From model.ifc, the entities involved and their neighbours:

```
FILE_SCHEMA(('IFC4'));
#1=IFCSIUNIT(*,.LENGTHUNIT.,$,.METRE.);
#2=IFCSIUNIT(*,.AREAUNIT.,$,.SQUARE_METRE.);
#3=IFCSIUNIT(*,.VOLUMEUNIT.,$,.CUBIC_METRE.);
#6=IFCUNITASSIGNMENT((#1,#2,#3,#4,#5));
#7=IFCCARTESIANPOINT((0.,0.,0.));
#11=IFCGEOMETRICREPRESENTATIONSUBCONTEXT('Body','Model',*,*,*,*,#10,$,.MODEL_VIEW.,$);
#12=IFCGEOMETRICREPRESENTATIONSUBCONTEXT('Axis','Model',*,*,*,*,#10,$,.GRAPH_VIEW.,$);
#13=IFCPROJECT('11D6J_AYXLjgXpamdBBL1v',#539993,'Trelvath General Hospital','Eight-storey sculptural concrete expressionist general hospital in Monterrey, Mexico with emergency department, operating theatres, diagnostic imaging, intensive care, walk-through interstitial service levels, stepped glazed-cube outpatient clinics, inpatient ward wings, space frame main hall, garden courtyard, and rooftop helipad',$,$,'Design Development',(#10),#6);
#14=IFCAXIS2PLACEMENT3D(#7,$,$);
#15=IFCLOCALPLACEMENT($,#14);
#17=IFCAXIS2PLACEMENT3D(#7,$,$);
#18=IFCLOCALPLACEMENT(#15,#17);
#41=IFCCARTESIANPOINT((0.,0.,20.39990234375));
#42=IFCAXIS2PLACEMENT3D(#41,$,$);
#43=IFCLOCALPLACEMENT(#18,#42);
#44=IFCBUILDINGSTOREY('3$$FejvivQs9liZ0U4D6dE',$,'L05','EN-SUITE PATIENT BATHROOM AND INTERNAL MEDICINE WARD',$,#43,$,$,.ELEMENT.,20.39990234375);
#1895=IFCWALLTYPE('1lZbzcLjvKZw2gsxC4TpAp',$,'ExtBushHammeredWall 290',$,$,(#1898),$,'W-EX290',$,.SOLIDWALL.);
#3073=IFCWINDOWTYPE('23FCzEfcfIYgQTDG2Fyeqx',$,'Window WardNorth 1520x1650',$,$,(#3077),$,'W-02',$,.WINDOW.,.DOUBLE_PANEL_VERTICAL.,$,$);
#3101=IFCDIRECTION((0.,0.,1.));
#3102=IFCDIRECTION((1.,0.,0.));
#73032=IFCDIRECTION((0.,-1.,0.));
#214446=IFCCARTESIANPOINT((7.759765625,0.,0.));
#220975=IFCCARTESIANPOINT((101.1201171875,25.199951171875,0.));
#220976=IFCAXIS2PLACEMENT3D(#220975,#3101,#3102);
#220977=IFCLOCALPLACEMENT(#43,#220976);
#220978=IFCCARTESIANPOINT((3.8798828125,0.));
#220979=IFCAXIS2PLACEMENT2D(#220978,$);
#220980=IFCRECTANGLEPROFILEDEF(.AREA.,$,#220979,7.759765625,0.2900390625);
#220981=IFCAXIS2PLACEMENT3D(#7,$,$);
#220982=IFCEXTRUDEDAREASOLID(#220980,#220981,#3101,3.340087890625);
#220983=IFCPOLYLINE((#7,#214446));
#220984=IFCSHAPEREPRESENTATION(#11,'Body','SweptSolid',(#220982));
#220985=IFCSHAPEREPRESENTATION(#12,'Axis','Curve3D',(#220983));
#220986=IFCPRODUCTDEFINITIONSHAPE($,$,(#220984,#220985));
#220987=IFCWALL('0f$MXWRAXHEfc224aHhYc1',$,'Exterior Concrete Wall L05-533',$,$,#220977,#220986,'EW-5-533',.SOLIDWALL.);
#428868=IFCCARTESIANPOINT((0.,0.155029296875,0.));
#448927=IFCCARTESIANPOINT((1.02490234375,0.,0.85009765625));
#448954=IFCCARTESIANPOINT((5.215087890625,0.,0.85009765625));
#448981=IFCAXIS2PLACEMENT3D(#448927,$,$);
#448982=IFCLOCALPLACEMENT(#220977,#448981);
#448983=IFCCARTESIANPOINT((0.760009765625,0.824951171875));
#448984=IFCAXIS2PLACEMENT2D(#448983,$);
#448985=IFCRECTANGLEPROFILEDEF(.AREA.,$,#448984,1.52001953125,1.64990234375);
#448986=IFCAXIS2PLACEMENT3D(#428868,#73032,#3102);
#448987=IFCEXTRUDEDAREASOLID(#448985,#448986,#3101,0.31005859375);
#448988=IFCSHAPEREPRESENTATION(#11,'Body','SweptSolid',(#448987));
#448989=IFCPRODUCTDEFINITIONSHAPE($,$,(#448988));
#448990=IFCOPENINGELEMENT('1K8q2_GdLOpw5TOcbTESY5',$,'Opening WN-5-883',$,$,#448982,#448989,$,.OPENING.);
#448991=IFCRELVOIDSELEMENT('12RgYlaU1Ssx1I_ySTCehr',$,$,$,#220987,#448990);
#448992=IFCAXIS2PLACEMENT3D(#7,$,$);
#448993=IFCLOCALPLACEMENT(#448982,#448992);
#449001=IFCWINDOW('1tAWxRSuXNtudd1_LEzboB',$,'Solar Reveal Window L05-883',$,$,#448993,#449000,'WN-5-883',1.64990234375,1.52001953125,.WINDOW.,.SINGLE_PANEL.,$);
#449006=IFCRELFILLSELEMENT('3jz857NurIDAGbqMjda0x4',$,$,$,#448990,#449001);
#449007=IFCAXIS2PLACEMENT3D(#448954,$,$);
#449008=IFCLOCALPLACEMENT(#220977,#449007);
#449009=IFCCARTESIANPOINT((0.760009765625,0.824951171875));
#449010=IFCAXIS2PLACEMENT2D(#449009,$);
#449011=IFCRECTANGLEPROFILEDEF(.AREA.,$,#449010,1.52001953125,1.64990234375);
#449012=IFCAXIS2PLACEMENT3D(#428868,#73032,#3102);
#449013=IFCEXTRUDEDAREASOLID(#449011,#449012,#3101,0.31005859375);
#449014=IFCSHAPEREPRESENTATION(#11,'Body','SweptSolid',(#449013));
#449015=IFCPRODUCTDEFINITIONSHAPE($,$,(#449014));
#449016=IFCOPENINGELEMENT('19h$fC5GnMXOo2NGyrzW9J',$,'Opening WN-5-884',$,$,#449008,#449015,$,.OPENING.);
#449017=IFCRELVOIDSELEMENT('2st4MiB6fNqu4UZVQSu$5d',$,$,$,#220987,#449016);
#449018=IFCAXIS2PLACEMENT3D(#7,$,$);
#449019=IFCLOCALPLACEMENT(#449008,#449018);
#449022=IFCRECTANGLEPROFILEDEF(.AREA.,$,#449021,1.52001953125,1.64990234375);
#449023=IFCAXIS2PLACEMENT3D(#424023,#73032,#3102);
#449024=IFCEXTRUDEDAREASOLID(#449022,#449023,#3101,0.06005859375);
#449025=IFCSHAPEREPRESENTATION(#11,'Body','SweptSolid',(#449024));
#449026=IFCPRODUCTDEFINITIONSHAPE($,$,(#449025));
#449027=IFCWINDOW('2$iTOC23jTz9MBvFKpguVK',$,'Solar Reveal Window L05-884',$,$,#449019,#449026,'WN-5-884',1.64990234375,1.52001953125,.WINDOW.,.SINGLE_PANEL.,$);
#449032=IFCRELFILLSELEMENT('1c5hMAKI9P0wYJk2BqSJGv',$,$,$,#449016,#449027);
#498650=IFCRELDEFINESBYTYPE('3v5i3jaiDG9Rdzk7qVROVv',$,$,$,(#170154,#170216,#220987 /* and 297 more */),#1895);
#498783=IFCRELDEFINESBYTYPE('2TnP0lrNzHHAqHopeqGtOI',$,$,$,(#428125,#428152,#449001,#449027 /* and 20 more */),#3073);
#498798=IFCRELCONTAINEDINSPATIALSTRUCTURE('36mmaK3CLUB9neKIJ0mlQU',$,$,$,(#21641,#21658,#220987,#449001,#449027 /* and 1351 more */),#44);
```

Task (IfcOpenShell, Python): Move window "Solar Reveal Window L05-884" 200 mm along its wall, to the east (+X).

```python
import ifcopenshell
import ifcopenshell.api.geometry
import ifcopenshell.util.placement

model = ifcopenshell.open("model.ifc")

window = model.by_id(449027)
opening = window.FillsVoids[0].RelatingOpeningElement
wall = opening.VoidsElements[0].RelatingBuildingElement

wall_matrix = ifcopenshell.util.placement.get_local_placement(wall.ObjectPlacement)
shift = wall_matrix[:3, 0] * 0.2
before = ifcopenshell.util.placement.get_local_placement(window.ObjectPlacement)[:3, 3].copy()

# The window is placed relative to its opening, so it follows when the opening moves.
matrix = ifcopenshell.util.placement.get_local_placement(opening.ObjectPlacement)
matrix[:3, 3] += shift
ifcopenshell.api.geometry.edit_object_placement(
    model, product=opening, matrix=matrix, is_si=False, should_transform_children=True
)

after = ifcopenshell.util.placement.get_local_placement(window.ObjectPlacement)[:3, 3]
print("window moved by", (after - before).round(3) + 0.0)

model.write("model_rev.ifc")
```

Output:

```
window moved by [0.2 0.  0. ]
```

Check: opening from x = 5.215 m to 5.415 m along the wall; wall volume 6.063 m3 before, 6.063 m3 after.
